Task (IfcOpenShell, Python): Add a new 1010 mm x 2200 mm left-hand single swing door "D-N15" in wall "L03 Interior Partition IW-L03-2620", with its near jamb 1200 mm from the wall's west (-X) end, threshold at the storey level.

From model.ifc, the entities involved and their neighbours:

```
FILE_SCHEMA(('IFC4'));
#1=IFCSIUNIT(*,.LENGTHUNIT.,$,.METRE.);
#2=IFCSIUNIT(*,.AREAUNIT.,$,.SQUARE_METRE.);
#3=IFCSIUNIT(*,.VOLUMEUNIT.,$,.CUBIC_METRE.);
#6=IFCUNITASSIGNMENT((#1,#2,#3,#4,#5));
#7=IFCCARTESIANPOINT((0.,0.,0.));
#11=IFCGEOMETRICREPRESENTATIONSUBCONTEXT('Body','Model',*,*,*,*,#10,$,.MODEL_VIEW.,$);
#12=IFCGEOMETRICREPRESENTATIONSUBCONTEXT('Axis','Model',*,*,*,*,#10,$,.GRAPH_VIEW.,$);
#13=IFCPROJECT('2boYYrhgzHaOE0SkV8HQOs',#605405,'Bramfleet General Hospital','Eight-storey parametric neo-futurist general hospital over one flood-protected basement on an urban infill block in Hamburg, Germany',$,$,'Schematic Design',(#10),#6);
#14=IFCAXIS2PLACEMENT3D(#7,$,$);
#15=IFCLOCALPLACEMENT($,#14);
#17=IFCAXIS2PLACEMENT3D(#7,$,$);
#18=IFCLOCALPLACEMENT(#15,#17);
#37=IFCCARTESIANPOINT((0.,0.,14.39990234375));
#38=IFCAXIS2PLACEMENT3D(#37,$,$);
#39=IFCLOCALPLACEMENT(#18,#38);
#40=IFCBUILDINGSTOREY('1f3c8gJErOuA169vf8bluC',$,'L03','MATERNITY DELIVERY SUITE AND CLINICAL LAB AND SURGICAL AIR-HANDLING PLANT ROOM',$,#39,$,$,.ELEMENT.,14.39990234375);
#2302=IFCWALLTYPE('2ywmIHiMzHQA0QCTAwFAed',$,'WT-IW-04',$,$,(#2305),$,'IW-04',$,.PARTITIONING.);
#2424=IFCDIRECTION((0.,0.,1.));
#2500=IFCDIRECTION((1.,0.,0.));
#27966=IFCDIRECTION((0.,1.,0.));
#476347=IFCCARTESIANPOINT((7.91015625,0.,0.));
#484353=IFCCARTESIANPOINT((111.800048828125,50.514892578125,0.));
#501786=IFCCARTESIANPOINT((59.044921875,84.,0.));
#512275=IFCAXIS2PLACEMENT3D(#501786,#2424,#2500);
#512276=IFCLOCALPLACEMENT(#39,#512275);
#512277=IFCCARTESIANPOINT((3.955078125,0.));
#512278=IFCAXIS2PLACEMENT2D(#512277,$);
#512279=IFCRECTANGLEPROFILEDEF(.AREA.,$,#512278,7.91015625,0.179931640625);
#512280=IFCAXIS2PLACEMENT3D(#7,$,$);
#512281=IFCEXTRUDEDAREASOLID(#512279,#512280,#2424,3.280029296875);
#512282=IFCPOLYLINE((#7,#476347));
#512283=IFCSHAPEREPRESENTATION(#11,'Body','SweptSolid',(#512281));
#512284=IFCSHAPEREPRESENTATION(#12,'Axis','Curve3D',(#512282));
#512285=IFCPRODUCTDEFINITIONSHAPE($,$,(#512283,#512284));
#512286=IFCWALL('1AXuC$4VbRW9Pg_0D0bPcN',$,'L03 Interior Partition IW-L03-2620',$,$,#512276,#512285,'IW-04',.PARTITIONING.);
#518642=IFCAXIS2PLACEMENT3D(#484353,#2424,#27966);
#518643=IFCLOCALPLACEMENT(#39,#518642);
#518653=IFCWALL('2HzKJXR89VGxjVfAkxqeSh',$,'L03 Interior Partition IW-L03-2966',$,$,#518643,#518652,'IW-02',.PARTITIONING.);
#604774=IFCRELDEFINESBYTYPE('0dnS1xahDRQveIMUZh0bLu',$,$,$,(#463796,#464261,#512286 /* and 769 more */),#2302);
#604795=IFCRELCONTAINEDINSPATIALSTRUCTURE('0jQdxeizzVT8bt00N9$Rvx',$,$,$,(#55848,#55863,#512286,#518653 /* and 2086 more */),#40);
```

```python
import numpy as np
import ifcopenshell
import ifcopenshell.api.feature
import ifcopenshell.api.geometry
import ifcopenshell.api.root
import ifcopenshell.api.spatial
import ifcopenshell.geom
import ifcopenshell.util.element
import ifcopenshell.util.placement
import ifcopenshell.util.representation
import ifcopenshell.util.shape
import ifcopenshell.util.unit

model = ifcopenshell.open("model.ifc")
unit_scale = ifcopenshell.util.unit.calculate_unit_scale(model)
settings = ifcopenshell.geom.settings()


def volume(element):
    """Net volume in cubic metres, openings subtracted."""
    shape = ifcopenshell.geom.create_shape(settings, element)
    return ifcopenshell.util.shape.get_volume(shape.geometry)


wall = model.by_guid("1AXuC$4VbRW9Pg_0D0bPcN")
storey = ifcopenshell.util.element.get_container(wall, ifc_class="IfcBuildingStorey")
context = ifcopenshell.util.representation.get_context(model, "Model", "Body", "MODEL_VIEW")
before = volume(wall)

width, height, from_end, sill = 1.01, 2.2, 1.2, 0.0  # metres

# The wall runs along its own X axis, and the end named is its -X end.
wall_shape = ifcopenshell.geom.create_shape(settings, wall)
x, y, z = ifcopenshell.util.shape.get_vertices(wall_shape.geometry).T
start = x.min() + from_end
face, thickness = float(y.min()), float(y.max() - y.min())
wall_matrix = ifcopenshell.util.placement.get_local_placement(wall.ObjectPlacement)
level = ifcopenshell.util.placement.get_local_placement(storey.ObjectPlacement)[2, 3]


def in_wall(x, y):
    """Placement at x, y metres in the wall's axes, at sill height."""
    matrix = wall_matrix.copy()
    matrix[:, 3] = wall_matrix @ np.array([x / unit_scale, y / unit_scale, 0.0, 1.0])
    matrix[2, 3] = level + sill / unit_scale
    return matrix


# Opening: a box that overshoots both wall faces by 50 mm.
opening = ifcopenshell.api.root.create_entity(model, ifc_class="IfcOpeningElement", predefined_type="OPENING")
box = ifcopenshell.api.geometry.add_wall_representation(
    model, context=context, length=width, height=height, thickness=thickness + 0.1
)
ifcopenshell.api.geometry.assign_representation(model, product=opening, representation=box)
ifcopenshell.api.geometry.edit_object_placement(model, product=opening, matrix=in_wall(start, face - 0.05), is_si=False)
ifcopenshell.api.feature.add_feature(model, feature=opening, element=wall)

door = ifcopenshell.api.root.create_entity(model, ifc_class="IfcDoor", name="D-N15", predefined_type="DOOR")
door.OverallWidth, door.OverallHeight = width / unit_scale, height / unit_scale
door.OperationType = "SINGLE_SWING_LEFT"
body = ifcopenshell.api.geometry.add_door_representation(
    model,
    context=context,
    overall_width=door.OverallWidth,
    overall_height=door.OverallHeight,
    operation_type="SINGLE_SWING_LEFT",
    lining_properties={"LiningDepth": thickness / unit_scale, "ThresholdDepth": thickness / unit_scale},
)
ifcopenshell.api.geometry.assign_representation(model, product=door, representation=body)
ifcopenshell.api.spatial.assign_container(model, products=[door], relating_structure=storey)
ifcopenshell.api.feature.add_filling(model, opening=opening, element=door)

# The lining spans the wall, so the door starts at the wall face.
ifcopenshell.api.geometry.edit_object_placement(model, product=door, matrix=in_wall(start, face), is_si=False)

after = volume(wall)

print(f"wall volume {before:.3f} -> {after:.3f} m3")

model.write("model_updated.ifc")
```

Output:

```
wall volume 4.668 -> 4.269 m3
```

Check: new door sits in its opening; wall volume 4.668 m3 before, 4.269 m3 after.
